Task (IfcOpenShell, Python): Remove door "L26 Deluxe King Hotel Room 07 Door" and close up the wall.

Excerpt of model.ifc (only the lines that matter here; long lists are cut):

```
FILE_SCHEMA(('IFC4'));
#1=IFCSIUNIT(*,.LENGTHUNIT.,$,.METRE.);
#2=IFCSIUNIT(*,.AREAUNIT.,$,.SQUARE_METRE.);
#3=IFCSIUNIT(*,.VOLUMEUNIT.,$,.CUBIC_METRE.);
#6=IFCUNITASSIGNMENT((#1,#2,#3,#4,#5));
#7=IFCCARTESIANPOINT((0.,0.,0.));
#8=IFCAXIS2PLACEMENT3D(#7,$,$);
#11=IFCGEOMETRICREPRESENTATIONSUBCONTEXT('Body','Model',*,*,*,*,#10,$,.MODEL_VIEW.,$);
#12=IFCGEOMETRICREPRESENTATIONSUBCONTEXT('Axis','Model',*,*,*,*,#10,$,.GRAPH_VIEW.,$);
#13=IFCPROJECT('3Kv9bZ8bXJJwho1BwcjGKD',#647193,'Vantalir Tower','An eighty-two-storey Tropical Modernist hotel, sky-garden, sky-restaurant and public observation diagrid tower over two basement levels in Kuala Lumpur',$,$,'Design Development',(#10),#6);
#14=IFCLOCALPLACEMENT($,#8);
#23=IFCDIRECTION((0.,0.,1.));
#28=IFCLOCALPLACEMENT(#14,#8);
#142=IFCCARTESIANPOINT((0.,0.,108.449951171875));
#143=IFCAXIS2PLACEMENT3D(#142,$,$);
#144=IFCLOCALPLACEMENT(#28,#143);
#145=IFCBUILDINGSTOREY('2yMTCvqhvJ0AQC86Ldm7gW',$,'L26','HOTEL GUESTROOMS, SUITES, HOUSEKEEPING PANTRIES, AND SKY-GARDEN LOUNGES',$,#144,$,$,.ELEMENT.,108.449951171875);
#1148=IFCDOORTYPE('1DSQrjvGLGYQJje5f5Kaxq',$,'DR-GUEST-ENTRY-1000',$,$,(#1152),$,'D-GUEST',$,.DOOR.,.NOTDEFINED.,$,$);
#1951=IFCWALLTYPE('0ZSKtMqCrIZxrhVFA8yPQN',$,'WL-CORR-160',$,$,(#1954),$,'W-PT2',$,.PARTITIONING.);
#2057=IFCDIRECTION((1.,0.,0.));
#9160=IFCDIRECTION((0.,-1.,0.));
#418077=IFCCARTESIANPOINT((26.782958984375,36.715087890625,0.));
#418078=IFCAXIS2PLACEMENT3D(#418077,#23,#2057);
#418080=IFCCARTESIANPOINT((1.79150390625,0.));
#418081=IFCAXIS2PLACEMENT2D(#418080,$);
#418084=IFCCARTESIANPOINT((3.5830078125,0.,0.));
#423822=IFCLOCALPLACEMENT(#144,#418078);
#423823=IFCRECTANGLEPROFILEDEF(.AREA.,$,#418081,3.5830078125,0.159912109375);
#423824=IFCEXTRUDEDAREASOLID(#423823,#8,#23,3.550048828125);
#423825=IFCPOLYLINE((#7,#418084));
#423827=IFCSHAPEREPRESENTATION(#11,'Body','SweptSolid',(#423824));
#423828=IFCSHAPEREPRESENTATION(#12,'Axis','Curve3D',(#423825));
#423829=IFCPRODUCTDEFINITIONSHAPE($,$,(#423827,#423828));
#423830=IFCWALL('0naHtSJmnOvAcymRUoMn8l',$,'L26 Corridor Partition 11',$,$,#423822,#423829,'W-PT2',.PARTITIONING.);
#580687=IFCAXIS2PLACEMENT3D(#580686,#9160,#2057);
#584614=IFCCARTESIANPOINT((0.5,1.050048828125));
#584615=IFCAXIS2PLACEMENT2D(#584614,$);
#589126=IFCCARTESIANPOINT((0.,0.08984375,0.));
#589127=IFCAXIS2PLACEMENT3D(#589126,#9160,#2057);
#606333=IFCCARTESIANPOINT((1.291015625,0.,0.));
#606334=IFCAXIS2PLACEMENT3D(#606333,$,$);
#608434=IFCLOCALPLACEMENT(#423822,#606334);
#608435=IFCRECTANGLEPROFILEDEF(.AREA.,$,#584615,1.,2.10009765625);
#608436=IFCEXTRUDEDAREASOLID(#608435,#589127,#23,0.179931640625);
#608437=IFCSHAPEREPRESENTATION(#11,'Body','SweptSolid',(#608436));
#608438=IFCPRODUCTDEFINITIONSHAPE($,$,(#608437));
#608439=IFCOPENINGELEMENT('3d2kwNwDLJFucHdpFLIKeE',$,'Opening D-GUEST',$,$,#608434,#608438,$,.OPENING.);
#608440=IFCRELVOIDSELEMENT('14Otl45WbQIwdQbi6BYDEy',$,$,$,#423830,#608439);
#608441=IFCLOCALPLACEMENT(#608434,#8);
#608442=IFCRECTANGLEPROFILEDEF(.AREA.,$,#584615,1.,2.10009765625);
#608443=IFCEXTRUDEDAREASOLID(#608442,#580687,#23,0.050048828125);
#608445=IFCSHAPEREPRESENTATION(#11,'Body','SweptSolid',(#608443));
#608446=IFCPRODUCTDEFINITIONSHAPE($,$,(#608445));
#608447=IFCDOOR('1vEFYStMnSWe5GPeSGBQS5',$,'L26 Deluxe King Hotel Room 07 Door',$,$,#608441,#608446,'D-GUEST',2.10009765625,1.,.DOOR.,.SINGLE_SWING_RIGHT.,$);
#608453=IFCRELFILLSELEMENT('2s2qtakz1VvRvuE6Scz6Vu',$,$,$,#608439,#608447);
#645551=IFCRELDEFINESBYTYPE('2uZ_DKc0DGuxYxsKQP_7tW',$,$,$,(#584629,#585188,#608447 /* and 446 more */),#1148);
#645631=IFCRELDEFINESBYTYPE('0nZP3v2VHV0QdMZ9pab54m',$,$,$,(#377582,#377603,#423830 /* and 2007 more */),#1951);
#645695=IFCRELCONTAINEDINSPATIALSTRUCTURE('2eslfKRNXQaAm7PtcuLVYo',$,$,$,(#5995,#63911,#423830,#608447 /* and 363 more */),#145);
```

```python
import ifcopenshell
import ifcopenshell.api.feature
import ifcopenshell.api.root
import ifcopenshell.geom
import ifcopenshell.util.shape

model = ifcopenshell.open("model.ifc")
settings = ifcopenshell.geom.settings()


def volume(element):
    """Net volume in cubic metres, openings subtracted."""
    shape = ifcopenshell.geom.create_shape(settings, element)
    return ifcopenshell.util.shape.get_volume(shape.geometry)


door = model.by_guid("1vEFYStMnSWe5GPeSGBQS5")
opening = door.FillsVoids[0].RelatingOpeningElement
wall = opening.VoidsElements[0].RelatingBuildingElement
before = volume(wall)

ifcopenshell.api.root.remove_product(model, product=door)
ifcopenshell.api.feature.remove_feature(model, feature=opening)

after = volume(wall)

print(f"wall volume {before:.3f} -> {after:.3f} m3")

model.write("model_rev.ifc")
```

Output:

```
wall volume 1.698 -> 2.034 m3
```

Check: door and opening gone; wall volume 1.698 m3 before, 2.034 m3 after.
